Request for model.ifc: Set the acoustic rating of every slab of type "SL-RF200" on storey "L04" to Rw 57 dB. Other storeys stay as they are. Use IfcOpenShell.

First a look at what the model holds.

```python
import ifcopenshell
import ifcopenshell.util.element

model = ifcopenshell.open("model.ifc")
print(model.schema)
storey = next(s for s in model.by_type("IfcBuildingStorey") if s.Name == "L04")
slabs = [e for e in ifcopenshell.util.element.get_decomposition(storey) if e.is_a("IfcSlab")]
seen = {}
for e in slabs:
    element_type = ifcopenshell.util.element.get_type(e)
    key = (element_type.Name if element_type != e and element_type else None, ifcopenshell.util.element.get_pset(e, "Pset_SlabCommon", "AcousticRating"))
    seen[key] = seen.get(key, 0) + 1
for (name, value), count in sorted(seen.items(), key=str):
    print(count, "x", name, "|", value)
```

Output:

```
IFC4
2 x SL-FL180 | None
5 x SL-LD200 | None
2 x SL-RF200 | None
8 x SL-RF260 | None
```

```python
import ifcopenshell
import ifcopenshell.api.pset
import ifcopenshell.util.element

model = ifcopenshell.open("model.ifc")

storey = next(s for s in model.by_type("IfcBuildingStorey") if s.Name == "L04")
slabs = [e for e in ifcopenshell.util.element.get_decomposition(storey) if e.is_a("IfcSlab")]

count = 0
for e in slabs:
    element_type = ifcopenshell.util.element.get_type(e)
    if element_type in (None, e) or element_type.Name != "SL-RF200":
        continue
    # add_pset returns the element's existing set when there is one.
    pset = ifcopenshell.api.pset.add_pset(model, product=e, name="Pset_SlabCommon")
    ifcopenshell.api.pset.edit_pset(model, pset=pset, properties={"AcousticRating": "Rw 57 dB"})
    count += 1

print(count, "slabs updated")

model.write("model_updated.ifc")
```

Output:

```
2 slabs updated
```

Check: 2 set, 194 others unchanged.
